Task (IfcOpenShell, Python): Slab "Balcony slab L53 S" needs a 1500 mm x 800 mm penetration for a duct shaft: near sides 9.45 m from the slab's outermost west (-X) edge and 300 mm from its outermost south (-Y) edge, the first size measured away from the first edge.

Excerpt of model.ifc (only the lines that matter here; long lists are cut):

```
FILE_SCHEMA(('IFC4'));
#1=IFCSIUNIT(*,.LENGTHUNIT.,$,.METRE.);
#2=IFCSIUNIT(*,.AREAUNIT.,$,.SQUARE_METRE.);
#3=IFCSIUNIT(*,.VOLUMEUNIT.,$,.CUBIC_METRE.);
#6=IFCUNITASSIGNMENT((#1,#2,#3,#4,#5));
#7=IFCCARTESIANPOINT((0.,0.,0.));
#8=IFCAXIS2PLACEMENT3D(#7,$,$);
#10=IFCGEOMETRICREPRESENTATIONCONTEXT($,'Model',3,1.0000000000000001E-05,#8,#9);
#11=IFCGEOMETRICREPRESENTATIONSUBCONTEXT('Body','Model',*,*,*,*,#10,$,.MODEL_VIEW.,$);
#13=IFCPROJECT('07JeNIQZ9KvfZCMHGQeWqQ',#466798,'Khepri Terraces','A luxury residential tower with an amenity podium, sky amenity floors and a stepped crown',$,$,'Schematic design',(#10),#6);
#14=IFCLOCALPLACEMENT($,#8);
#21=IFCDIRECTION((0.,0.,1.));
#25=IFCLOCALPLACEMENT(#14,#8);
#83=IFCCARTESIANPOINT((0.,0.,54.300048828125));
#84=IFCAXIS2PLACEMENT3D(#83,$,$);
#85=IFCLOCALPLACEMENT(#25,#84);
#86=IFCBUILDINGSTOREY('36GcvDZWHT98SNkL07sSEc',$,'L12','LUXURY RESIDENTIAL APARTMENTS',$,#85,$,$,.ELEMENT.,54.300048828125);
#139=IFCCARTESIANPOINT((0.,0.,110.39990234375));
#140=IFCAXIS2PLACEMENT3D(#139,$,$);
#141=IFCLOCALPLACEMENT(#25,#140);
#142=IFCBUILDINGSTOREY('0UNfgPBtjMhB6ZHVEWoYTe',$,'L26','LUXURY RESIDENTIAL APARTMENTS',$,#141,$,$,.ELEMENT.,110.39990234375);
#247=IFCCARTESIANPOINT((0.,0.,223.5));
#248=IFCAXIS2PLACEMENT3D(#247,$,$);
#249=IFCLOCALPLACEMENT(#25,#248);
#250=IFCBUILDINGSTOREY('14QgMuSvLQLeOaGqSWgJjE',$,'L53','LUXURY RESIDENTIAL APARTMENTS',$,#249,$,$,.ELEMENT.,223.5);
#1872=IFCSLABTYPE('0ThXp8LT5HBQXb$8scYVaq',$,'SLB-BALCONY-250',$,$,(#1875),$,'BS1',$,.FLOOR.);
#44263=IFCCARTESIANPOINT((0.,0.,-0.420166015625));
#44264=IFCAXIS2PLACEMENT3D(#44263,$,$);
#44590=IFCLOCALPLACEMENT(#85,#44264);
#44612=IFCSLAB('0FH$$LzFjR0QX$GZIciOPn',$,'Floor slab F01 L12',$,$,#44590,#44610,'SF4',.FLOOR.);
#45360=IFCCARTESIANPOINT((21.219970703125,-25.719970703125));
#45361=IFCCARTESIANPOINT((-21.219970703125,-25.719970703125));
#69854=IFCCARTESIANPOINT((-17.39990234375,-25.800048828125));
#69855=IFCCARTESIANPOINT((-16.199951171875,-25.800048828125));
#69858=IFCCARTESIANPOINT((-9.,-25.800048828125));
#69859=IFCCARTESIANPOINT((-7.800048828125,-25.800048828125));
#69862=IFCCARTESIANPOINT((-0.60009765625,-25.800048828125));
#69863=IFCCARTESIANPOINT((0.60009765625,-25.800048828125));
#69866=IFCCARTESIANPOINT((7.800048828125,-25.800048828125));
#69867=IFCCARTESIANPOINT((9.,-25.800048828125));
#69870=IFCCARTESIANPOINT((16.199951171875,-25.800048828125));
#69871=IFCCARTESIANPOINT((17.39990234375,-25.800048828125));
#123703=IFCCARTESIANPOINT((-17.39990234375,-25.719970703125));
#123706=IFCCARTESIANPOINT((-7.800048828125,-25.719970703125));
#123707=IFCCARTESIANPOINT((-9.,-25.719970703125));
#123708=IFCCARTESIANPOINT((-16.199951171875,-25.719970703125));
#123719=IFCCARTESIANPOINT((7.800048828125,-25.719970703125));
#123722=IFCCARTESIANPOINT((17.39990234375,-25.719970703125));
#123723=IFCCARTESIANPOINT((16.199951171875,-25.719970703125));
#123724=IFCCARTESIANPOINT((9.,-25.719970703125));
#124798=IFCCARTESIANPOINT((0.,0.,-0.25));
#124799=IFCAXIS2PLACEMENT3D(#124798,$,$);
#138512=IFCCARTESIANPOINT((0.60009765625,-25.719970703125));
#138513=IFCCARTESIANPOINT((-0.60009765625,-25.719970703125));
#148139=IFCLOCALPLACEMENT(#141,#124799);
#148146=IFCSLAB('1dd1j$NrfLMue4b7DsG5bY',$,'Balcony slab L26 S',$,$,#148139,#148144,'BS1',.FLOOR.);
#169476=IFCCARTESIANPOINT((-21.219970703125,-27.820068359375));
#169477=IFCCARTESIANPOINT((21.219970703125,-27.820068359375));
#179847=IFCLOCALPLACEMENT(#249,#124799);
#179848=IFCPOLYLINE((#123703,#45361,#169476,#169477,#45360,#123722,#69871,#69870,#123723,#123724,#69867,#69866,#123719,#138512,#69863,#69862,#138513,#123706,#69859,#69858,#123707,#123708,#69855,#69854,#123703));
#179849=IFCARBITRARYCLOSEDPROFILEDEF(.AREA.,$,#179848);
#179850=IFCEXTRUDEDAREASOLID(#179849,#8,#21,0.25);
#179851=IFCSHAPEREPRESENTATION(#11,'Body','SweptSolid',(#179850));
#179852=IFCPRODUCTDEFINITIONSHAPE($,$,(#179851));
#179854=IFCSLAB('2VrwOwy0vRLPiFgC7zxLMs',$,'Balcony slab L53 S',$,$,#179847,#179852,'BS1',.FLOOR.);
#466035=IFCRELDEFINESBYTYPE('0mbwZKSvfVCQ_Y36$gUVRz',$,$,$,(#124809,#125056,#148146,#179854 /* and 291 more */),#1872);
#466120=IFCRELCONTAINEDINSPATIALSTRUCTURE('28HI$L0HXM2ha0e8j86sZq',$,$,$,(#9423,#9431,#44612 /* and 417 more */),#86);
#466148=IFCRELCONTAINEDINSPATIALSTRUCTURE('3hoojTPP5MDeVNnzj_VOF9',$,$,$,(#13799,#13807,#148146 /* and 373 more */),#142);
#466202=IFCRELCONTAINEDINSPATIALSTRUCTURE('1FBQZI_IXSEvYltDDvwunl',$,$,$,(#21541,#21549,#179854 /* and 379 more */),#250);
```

```python
import numpy as np
import ifcopenshell
import ifcopenshell.api.feature
import ifcopenshell.api.geometry
import ifcopenshell.api.root
import ifcopenshell.geom
import ifcopenshell.util.placement
import ifcopenshell.util.representation
import ifcopenshell.util.shape
import ifcopenshell.util.unit

model = ifcopenshell.open("model.ifc")
unit_scale = ifcopenshell.util.unit.calculate_unit_scale(model)
settings = ifcopenshell.geom.settings()


def volume(element):
    """Net volume in cubic metres, openings subtracted."""
    shape = ifcopenshell.geom.create_shape(settings, element)
    return ifcopenshell.util.shape.get_volume(shape.geometry)


slab = model.by_guid("2VrwOwy0vRLPiFgC7zxLMs")
before = volume(slab)

# Extent in the slab's own axes, in metres. The edges named are its -X and -Y sides.
slab_shape = ifcopenshell.geom.create_shape(settings, slab)
vertices = ifcopenshell.util.shape.get_vertices(slab_shape.geometry)
x_min, y_min, bottom = vertices.min(axis=0)
top = vertices[:, 2].max()

opening = ifcopenshell.api.root.create_entity(model, ifc_class="IfcOpeningElement", name="Duct shaft opening", predefined_type="OPENING")
context = ifcopenshell.util.representation.get_context(model, "Model", "Body", "MODEL_VIEW")
width, depth = 1.5, 0.8
outline = [(0.0, 0.0), (width, 0.0), (width, depth), (0.0, depth), (0.0, 0.0)]
# Overshoot both faces by 50 mm so the cut is clean.
shape = ifcopenshell.api.geometry.add_slab_representation(
    model, context=context, depth=top - bottom + 0.1, polyline=outline
)
ifcopenshell.api.geometry.assign_representation(model, product=opening, representation=shape)

matrix = ifcopenshell.util.placement.get_local_placement(slab.ObjectPlacement)
matrix[:, 3] = matrix @ np.append(np.array([x_min + 9.45, y_min + 0.3, bottom - 0.05]) / unit_scale, 1.0)
ifcopenshell.api.geometry.edit_object_placement(model, product=opening, matrix=matrix, is_si=False)
ifcopenshell.api.feature.add_feature(model, feature=opening, element=slab)

after = volume(slab)

print(f"slab volume {before:.3f} -> {after:.3f} m3")

model.write("model_edited.ifc")
```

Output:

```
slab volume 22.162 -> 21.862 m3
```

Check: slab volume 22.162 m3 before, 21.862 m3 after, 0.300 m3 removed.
